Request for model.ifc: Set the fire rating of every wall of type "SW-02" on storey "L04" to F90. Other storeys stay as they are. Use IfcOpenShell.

First a look at what the model holds.

```python
import ifcopenshell
import ifcopenshell.util.element

model = ifcopenshell.open("model.ifc")
print(model.schema)
storey = next(s for s in model.by_type("IfcBuildingStorey") if s.Name == "L04")
walls = [e for e in ifcopenshell.util.element.get_decomposition(storey) if e.is_a("IfcWall")]
seen = {}
for e in walls:
    element_type = ifcopenshell.util.element.get_type(e)
    key = (element_type.Name if element_type != e and element_type else None, ifcopenshell.util.element.get_pset(e, "Pset_WallCommon", "FireRating"))
    seen[key] = seen.get(key, 0) + 1
for (name, value), count in sorted(seen.items(), key=str):
    print(count, "x", name, "|", value)
```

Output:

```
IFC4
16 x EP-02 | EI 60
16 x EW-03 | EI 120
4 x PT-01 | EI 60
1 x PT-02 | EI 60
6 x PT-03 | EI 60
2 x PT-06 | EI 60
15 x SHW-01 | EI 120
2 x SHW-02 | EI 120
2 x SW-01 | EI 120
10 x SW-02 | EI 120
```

```python
import ifcopenshell
import ifcopenshell.api.pset
import ifcopenshell.util.element

model = ifcopenshell.open("model.ifc")

storey = next(s for s in model.by_type("IfcBuildingStorey") if s.Name == "L04")
walls = [e for e in ifcopenshell.util.element.get_decomposition(storey) if e.is_a("IfcWall")]

count = 0
for e in walls:
    element_type = ifcopenshell.util.element.get_type(e)
    if element_type in (None, e) or element_type.Name != "SW-02":
        continue
    # add_pset returns the element's existing set when there is one.
    pset = ifcopenshell.api.pset.add_pset(model, product=e, name="Pset_WallCommon")
    ifcopenshell.api.pset.edit_pset(model, pset=pset, properties={"FireRating": "F90"})
    count += 1

print(count, "walls updated")

model.write("model-out.ifc")
```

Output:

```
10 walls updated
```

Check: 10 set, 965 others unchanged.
